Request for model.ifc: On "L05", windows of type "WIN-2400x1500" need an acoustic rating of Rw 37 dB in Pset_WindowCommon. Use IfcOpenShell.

First a look at what the model holds.

```python
import ifcopenshell
import ifcopenshell.util.element

model = ifcopenshell.open("model.ifc")
print(model.schema)
storey = next(s for s in model.by_type("IfcBuildingStorey") if s.Name == "L05")
windows = [e for e in ifcopenshell.util.element.get_decomposition(storey) if e.is_a("IfcWindow")]
seen = {}
for e in windows:
    element_type = ifcopenshell.util.element.get_type(e)
    key = (element_type.Name if element_type != e and element_type else None, ifcopenshell.util.element.get_pset(e, "Pset_WindowCommon", "AcousticRating"))
    seen[key] = seen.get(key, 0) + 1
for (name, value), count in sorted(seen.items(), key=str):
    print(count, "x", name, "|", value)
```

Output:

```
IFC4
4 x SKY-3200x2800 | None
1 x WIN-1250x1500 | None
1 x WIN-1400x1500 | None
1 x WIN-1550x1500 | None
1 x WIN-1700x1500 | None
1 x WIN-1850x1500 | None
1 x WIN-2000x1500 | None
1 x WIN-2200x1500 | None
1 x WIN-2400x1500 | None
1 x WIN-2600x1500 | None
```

```python
import ifcopenshell
import ifcopenshell.api.pset
import ifcopenshell.util.element

model = ifcopenshell.open("model.ifc")

storey = next(s for s in model.by_type("IfcBuildingStorey") if s.Name == "L05")
windows = [e for e in ifcopenshell.util.element.get_decomposition(storey) if e.is_a("IfcWindow")]

count = 0
for e in windows:
    element_type = ifcopenshell.util.element.get_type(e)
    if element_type in (None, e) or element_type.Name != "WIN-2400x1500":
        continue
    # add_pset returns the element's existing set when there is one.
    pset = ifcopenshell.api.pset.add_pset(model, product=e, name="Pset_WindowCommon")
    ifcopenshell.api.pset.edit_pset(model, pset=pset, properties={"AcousticRating": "Rw 37 dB"})
    count += 1

print(count, "windows updated")

model.write("model-out.ifc")
```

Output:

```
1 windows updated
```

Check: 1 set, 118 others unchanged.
